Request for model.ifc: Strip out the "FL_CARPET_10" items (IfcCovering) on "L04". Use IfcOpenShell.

First a look at what the model holds.

```python
import ifcopenshell
import ifcopenshell.util.element

model = ifcopenshell.open("model.ifc")
print(model.schema)
storey = next(s for s in model.by_type("IfcBuildingStorey") if s.Name == "L04")
coverings = [e for e in ifcopenshell.util.element.get_decomposition(storey) if e.is_a("IfcCovering")]
seen = {}
for e in coverings:
    element_type = ifcopenshell.util.element.get_type(e)
    name = element_type.Name if element_type not in (None, e) else None
    seen[name] = seen.get(name, 0) + 1
for name, count in sorted(seen.items(), key=str):
    print(count, "x", name)
```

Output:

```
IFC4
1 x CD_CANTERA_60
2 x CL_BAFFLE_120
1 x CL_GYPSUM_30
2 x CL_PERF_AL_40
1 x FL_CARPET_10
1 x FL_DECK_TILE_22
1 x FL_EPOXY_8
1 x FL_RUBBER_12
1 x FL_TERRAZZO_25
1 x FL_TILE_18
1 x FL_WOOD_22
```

```python
import ifcopenshell
import ifcopenshell.api.root
import ifcopenshell.util.element

model = ifcopenshell.open("model.ifc")

storey = next(s for s in model.by_type("IfcBuildingStorey") if s.Name == "L04")
coverings = [e for e in ifcopenshell.util.element.get_decomposition(storey) if e.is_a("IfcCovering")]
targets = [e for e in coverings if (t := ifcopenshell.util.element.get_type(e)) not in (None, e) and t.Name == "FL_CARPET_10"]

for e in targets:
    ifcopenshell.api.root.remove_product(model, product=e)
print(len(targets), "removed")

model.write("model_updated.ifc")
```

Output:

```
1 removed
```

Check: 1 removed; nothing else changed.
